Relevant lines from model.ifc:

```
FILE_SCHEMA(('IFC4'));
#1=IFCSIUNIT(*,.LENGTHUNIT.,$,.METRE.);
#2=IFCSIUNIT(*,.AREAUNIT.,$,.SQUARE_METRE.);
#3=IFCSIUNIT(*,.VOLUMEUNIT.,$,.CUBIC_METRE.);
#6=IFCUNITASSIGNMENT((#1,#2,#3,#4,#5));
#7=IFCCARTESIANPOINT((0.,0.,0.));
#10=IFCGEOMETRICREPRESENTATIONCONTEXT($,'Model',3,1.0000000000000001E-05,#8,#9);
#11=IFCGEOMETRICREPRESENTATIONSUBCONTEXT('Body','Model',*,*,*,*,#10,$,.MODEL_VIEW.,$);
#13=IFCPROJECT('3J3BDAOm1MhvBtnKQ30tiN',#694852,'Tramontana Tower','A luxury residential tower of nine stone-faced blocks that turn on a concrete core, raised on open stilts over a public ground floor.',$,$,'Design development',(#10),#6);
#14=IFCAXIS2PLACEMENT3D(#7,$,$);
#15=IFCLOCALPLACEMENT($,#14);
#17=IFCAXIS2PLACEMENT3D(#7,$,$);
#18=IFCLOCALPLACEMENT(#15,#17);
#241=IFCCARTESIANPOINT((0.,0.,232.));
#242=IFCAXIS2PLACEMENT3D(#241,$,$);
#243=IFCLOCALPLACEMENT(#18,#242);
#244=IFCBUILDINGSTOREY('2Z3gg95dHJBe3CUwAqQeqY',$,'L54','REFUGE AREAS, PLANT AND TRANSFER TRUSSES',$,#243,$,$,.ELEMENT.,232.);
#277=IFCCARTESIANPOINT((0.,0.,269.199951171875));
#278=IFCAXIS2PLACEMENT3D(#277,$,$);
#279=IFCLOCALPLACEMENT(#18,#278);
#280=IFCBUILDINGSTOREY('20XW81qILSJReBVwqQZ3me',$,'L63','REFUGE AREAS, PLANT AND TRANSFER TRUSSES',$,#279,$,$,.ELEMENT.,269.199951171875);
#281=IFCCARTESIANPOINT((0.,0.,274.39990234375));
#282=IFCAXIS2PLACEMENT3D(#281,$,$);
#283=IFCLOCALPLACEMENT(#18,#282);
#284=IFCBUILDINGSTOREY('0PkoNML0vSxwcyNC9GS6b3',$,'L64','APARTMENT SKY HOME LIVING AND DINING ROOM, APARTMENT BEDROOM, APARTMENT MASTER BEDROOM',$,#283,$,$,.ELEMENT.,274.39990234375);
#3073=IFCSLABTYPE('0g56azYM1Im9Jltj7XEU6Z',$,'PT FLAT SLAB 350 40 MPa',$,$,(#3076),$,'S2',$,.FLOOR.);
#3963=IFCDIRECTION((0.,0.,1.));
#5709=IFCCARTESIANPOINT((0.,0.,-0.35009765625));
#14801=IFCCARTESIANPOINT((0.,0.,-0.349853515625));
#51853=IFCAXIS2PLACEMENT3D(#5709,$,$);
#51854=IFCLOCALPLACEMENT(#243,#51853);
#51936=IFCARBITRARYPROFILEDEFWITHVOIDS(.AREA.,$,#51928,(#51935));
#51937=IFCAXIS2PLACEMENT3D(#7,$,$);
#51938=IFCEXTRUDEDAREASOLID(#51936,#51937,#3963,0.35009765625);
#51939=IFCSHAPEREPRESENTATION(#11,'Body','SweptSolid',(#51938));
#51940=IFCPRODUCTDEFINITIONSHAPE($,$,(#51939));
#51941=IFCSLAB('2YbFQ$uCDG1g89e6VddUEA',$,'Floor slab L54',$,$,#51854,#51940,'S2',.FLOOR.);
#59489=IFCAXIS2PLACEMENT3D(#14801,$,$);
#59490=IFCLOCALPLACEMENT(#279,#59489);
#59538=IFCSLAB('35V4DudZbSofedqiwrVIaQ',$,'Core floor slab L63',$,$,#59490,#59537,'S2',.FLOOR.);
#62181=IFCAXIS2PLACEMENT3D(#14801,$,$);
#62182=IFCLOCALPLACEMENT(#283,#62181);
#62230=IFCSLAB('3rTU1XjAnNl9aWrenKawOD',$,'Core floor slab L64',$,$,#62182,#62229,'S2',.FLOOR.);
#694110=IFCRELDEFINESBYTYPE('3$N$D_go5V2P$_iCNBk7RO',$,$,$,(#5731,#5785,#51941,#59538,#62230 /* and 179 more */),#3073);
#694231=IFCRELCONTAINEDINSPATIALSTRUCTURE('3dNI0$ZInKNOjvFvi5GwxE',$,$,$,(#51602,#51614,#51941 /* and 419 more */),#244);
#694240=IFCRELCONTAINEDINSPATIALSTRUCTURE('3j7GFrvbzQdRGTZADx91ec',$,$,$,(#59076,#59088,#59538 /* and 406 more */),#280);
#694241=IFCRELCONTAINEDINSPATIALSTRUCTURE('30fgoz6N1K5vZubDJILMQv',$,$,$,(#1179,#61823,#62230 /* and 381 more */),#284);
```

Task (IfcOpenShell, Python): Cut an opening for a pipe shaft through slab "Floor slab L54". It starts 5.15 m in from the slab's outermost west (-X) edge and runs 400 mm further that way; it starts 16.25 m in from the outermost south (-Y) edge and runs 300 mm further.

```python
import numpy as np
import ifcopenshell
import ifcopenshell.api.feature
import ifcopenshell.api.geometry
import ifcopenshell.api.root
import ifcopenshell.geom
import ifcopenshell.util.placement
import ifcopenshell.util.representation
import ifcopenshell.util.shape
import ifcopenshell.util.unit

model = ifcopenshell.open("model.ifc")
unit_scale = ifcopenshell.util.unit.calculate_unit_scale(model)
settings = ifcopenshell.geom.settings()


def volume(element):
    """Net volume in cubic metres, openings subtracted."""
    shape = ifcopenshell.geom.create_shape(settings, element)
    return ifcopenshell.util.shape.get_volume(shape.geometry)


slab = model.by_guid("2YbFQ$uCDG1g89e6VddUEA")
before = volume(slab)

# Extent in the slab's own axes, in metres. The edges named are its -X and -Y sides.
slab_shape = ifcopenshell.geom.create_shape(settings, slab)
vertices = ifcopenshell.util.shape.get_vertices(slab_shape.geometry)
x_min, y_min, bottom = vertices.min(axis=0)
top = vertices[:, 2].max()

opening = ifcopenshell.api.root.create_entity(model, ifc_class="IfcOpeningElement", name="Pipe shaft opening", predefined_type="OPENING")
context = ifcopenshell.util.representation.get_context(model, "Model", "Body", "MODEL_VIEW")
width, depth = 0.4, 0.3
outline = [(0.0, 0.0), (width, 0.0), (width, depth), (0.0, depth), (0.0, 0.0)]
# Overshoot both faces by 50 mm so the cut is clean.
shape = ifcopenshell.api.geometry.add_slab_representation(
    model, context=context, depth=top - bottom + 0.1, polyline=outline
)
ifcopenshell.api.geometry.assign_representation(model, product=opening, representation=shape)

matrix = ifcopenshell.util.placement.get_local_placement(slab.ObjectPlacement)
matrix[:, 3] = matrix @ np.append(np.array([x_min + 5.15, y_min + 16.25, bottom - 0.05]) / unit_scale, 1.0)
ifcopenshell.api.geometry.edit_object_placement(model, product=opening, matrix=matrix, is_si=False)
ifcopenshell.api.feature.add_feature(model, feature=opening, element=slab)

after = volume(slab)

print(f"slab volume {before:.3f} -> {after:.3f} m3")

model.write("model-out.ifc")
```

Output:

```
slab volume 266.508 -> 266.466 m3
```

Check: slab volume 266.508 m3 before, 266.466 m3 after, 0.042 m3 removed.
